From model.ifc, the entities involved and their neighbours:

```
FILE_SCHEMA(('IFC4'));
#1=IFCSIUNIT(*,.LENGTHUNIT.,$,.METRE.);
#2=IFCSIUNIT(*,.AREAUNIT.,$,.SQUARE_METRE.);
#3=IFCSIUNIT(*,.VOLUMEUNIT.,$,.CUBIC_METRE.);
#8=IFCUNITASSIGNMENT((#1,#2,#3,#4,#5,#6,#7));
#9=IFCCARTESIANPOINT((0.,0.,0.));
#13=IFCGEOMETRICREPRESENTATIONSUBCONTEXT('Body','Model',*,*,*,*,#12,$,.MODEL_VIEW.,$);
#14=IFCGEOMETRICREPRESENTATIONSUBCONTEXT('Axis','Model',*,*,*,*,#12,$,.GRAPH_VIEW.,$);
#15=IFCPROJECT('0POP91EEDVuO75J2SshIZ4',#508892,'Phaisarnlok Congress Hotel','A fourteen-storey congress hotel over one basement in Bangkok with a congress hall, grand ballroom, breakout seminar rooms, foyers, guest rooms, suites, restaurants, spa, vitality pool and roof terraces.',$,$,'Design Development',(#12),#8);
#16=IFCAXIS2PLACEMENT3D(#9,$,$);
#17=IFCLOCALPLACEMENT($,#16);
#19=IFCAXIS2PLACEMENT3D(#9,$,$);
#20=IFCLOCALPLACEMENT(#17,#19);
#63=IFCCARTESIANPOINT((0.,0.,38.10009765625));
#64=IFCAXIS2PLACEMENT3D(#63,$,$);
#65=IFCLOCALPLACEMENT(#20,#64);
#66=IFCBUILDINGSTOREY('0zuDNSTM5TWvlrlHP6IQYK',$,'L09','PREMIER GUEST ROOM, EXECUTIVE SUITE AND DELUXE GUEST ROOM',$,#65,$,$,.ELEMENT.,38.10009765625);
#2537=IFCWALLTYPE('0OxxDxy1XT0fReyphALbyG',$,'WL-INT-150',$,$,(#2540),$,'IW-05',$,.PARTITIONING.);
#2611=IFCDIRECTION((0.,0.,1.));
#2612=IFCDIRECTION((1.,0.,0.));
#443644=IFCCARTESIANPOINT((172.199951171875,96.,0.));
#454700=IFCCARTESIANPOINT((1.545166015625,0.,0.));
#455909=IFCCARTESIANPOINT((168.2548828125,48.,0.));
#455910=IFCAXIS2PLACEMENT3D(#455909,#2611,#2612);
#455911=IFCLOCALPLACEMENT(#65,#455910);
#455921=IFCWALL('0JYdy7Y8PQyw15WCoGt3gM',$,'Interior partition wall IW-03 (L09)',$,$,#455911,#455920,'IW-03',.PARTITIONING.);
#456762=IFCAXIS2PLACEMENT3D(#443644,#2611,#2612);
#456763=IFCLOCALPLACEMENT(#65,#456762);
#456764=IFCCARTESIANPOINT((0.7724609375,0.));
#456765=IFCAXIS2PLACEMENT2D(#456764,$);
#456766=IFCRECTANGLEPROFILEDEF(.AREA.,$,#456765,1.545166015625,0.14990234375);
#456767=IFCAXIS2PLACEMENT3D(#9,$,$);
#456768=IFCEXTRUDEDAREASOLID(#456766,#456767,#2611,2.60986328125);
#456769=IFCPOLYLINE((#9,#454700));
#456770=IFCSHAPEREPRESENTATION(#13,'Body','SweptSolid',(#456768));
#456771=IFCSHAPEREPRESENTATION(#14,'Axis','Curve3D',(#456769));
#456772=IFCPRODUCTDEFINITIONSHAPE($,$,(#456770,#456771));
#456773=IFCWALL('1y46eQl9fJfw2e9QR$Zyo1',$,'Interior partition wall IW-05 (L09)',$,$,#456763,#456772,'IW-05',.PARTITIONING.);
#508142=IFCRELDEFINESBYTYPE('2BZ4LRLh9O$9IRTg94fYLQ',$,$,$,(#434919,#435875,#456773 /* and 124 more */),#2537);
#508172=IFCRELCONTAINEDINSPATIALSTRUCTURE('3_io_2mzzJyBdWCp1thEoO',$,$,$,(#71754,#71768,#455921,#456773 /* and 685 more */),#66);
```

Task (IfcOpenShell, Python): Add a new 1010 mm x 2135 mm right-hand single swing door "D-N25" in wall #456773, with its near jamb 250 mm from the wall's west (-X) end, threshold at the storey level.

```python
import numpy as np
import ifcopenshell
import ifcopenshell.api.feature
import ifcopenshell.api.geometry
import ifcopenshell.api.root
import ifcopenshell.api.spatial
import ifcopenshell.geom
import ifcopenshell.util.element
import ifcopenshell.util.placement
import ifcopenshell.util.representation
import ifcopenshell.util.shape
import ifcopenshell.util.unit

model = ifcopenshell.open("model.ifc")
unit_scale = ifcopenshell.util.unit.calculate_unit_scale(model)
settings = ifcopenshell.geom.settings()


def volume(element):
    """Net volume in cubic metres, openings subtracted."""
    shape = ifcopenshell.geom.create_shape(settings, element)
    return ifcopenshell.util.shape.get_volume(shape.geometry)


wall = model.by_id(456773)
storey = ifcopenshell.util.element.get_container(wall, ifc_class="IfcBuildingStorey")
context = ifcopenshell.util.representation.get_context(model, "Model", "Body", "MODEL_VIEW")
before = volume(wall)

width, height, from_end, sill = 1.01, 2.135, 0.25, 0.0  # metres

# The wall runs along its own X axis, and the end named is its -X end.
wall_shape = ifcopenshell.geom.create_shape(settings, wall)
x, y, z = ifcopenshell.util.shape.get_vertices(wall_shape.geometry).T
start = x.min() + from_end
face, thickness = float(y.min()), float(y.max() - y.min())
wall_matrix = ifcopenshell.util.placement.get_local_placement(wall.ObjectPlacement)
level = ifcopenshell.util.placement.get_local_placement(storey.ObjectPlacement)[2, 3]


def in_wall(x, y):
    """Placement at x, y metres in the wall's axes, at sill height."""
    matrix = wall_matrix.copy()
    matrix[:, 3] = wall_matrix @ np.array([x / unit_scale, y / unit_scale, 0.0, 1.0])
    matrix[2, 3] = level + sill / unit_scale
    return matrix


# Opening: a box that overshoots both wall faces by 50 mm.
opening = ifcopenshell.api.root.create_entity(model, ifc_class="IfcOpeningElement", predefined_type="OPENING")
box = ifcopenshell.api.geometry.add_wall_representation(
    model, context=context, length=width, height=height, thickness=thickness + 0.1
)
ifcopenshell.api.geometry.assign_representation(model, product=opening, representation=box)
ifcopenshell.api.geometry.edit_object_placement(model, product=opening, matrix=in_wall(start, face - 0.05), is_si=False)
ifcopenshell.api.feature.add_feature(model, feature=opening, element=wall)

door = ifcopenshell.api.root.create_entity(model, ifc_class="IfcDoor", name="D-N25", predefined_type="DOOR")
door.OverallWidth, door.OverallHeight = width / unit_scale, height / unit_scale
door.OperationType = "SINGLE_SWING_RIGHT"
body = ifcopenshell.api.geometry.add_door_representation(
    model,
    context=context,
    overall_width=door.OverallWidth,
    overall_height=door.OverallHeight,
    operation_type="SINGLE_SWING_RIGHT",
    lining_properties={"LiningDepth": thickness / unit_scale, "ThresholdDepth": thickness / unit_scale},
)
ifcopenshell.api.geometry.assign_representation(model, product=door, representation=body)
ifcopenshell.api.spatial.assign_container(model, products=[door], relating_structure=storey)
ifcopenshell.api.feature.add_filling(model, opening=opening, element=door)

# The lining spans the wall, so the door starts at the wall face.
ifcopenshell.api.geometry.edit_object_placement(model, product=door, matrix=in_wall(start, face), is_si=False)

after = volume(wall)

print(f"wall volume {before:.3f} -> {after:.3f} m3")

model.write("model_rev.ifc")
```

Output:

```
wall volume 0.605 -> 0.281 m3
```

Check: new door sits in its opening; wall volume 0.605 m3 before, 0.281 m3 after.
